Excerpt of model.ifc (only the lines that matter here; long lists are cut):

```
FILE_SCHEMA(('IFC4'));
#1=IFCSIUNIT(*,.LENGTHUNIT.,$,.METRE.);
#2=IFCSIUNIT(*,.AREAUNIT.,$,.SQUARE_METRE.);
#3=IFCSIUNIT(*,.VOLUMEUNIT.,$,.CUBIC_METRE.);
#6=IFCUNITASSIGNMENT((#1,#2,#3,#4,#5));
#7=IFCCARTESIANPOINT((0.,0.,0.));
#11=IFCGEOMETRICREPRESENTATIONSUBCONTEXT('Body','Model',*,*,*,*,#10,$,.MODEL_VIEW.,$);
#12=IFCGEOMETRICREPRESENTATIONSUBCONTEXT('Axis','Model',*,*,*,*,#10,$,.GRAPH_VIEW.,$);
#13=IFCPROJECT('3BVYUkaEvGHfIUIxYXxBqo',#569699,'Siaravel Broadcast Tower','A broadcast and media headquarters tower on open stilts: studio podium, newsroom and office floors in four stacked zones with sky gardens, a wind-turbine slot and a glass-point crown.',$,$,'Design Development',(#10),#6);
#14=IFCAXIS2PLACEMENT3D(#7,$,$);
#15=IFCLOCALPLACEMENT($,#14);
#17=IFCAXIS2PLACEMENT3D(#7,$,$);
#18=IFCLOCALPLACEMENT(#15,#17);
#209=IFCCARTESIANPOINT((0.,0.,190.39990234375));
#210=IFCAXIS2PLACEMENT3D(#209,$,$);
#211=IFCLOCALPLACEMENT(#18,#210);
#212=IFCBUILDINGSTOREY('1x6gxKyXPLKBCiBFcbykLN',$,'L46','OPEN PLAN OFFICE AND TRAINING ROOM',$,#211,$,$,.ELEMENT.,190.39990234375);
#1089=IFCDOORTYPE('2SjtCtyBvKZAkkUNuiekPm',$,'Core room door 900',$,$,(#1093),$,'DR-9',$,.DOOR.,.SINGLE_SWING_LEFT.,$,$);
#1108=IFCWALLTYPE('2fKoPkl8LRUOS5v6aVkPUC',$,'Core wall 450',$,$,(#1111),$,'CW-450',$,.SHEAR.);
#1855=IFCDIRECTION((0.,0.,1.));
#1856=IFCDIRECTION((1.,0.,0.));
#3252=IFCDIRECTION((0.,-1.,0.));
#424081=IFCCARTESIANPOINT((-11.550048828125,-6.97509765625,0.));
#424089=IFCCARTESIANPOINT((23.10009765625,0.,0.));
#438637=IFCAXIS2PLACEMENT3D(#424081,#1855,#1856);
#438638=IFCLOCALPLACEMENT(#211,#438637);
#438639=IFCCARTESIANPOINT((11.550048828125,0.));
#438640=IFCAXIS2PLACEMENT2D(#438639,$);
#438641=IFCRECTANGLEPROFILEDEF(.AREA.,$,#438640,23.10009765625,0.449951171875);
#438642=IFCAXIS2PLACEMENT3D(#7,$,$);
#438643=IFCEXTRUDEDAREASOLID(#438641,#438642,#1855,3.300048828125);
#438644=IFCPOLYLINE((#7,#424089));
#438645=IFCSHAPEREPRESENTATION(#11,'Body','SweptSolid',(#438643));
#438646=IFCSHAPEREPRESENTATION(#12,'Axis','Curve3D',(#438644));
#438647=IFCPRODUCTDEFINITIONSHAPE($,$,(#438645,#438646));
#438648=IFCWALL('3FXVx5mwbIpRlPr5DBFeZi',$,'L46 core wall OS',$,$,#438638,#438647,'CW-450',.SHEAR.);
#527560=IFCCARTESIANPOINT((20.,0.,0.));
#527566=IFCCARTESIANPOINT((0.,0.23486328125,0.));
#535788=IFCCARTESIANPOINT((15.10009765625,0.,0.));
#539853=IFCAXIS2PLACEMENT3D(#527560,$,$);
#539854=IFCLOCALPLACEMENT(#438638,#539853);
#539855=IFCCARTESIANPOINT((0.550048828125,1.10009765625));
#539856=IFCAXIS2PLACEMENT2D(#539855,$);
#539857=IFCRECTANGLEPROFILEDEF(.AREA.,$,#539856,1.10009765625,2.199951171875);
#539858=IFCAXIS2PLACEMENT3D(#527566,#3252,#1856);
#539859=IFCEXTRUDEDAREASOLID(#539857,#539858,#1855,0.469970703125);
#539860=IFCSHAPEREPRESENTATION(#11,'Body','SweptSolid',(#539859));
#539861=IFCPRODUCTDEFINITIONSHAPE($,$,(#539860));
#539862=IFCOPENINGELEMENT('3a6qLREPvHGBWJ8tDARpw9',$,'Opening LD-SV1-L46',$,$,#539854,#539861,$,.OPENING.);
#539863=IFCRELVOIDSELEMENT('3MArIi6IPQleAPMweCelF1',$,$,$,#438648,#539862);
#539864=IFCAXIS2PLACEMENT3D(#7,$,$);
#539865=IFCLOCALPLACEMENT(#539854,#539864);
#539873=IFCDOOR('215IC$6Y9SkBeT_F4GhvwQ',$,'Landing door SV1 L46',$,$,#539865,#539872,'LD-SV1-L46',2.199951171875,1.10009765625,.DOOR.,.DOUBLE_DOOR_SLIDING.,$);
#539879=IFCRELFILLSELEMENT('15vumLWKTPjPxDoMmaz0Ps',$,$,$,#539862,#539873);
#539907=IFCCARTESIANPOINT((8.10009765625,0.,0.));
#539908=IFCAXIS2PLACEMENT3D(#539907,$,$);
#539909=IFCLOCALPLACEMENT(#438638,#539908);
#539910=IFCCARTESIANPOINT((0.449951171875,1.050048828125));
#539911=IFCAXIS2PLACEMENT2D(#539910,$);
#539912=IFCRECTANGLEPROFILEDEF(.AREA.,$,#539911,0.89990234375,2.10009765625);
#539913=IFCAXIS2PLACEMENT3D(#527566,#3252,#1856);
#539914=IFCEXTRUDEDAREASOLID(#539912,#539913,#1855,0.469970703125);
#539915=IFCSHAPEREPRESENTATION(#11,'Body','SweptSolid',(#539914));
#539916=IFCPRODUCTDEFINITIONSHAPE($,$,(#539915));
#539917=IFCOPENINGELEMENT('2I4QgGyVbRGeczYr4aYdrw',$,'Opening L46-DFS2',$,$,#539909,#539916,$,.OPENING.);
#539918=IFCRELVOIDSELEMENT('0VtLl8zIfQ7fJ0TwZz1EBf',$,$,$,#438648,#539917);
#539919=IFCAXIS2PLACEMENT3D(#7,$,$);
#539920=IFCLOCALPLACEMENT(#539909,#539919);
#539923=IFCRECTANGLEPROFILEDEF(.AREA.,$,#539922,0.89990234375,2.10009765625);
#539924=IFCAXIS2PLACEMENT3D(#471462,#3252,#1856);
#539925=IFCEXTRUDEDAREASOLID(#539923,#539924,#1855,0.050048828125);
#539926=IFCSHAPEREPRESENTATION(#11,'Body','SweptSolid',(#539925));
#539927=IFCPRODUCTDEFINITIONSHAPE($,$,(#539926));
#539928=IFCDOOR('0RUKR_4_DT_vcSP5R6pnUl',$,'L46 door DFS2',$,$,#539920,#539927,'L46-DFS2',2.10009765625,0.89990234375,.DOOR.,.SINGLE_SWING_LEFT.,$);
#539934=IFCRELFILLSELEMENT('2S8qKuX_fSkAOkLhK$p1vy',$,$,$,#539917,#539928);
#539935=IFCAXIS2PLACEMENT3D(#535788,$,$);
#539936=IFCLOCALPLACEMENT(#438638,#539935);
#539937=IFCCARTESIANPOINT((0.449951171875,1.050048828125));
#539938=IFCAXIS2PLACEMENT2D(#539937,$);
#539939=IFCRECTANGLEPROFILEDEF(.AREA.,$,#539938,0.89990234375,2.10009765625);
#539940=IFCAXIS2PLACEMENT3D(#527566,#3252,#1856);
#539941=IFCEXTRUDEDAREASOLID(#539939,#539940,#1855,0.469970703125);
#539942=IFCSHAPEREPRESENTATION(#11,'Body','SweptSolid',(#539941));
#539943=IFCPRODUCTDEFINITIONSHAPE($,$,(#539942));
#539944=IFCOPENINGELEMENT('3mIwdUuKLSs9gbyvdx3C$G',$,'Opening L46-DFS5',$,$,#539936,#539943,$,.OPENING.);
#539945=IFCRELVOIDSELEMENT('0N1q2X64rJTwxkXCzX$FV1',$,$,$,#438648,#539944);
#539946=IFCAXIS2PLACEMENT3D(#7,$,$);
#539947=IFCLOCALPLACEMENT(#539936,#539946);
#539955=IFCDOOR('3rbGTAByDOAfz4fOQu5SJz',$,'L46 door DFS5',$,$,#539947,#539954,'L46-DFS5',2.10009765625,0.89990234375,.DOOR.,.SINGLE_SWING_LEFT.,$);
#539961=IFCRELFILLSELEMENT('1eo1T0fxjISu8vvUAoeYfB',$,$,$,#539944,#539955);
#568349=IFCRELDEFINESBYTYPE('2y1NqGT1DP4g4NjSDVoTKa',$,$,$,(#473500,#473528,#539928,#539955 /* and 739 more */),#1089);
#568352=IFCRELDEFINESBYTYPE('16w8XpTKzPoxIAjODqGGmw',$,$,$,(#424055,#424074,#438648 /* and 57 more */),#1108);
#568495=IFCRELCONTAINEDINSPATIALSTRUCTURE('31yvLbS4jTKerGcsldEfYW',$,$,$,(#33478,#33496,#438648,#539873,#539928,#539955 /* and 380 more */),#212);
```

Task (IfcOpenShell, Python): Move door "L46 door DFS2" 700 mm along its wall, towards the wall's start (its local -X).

```python
import ifcopenshell
import ifcopenshell.api.geometry
import ifcopenshell.util.placement

model = ifcopenshell.open("model.ifc")

door = model.by_guid("0RUKR_4_DT_vcSP5R6pnUl")
opening = door.FillsVoids[0].RelatingOpeningElement
wall = opening.VoidsElements[0].RelatingBuildingElement

wall_matrix = ifcopenshell.util.placement.get_local_placement(wall.ObjectPlacement)
shift = wall_matrix[:3, 0] * -0.7
before = ifcopenshell.util.placement.get_local_placement(door.ObjectPlacement)[:3, 3].copy()

# The door is placed relative to its opening, so it follows when the opening moves.
matrix = ifcopenshell.util.placement.get_local_placement(opening.ObjectPlacement)
matrix[:3, 3] += shift
ifcopenshell.api.geometry.edit_object_placement(
    model, product=opening, matrix=matrix, is_si=False, should_transform_children=True
)

after = ifcopenshell.util.placement.get_local_placement(door.ObjectPlacement)[:3, 3]
print("door moved by", (after - before).round(3) + 0.0)

model.write("model_v2.ifc")
```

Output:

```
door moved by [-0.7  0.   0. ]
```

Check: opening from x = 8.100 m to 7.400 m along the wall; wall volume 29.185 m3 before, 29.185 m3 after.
